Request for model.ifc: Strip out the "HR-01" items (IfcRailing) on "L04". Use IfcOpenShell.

First a look at what the model holds.

```python
import ifcopenshell
import ifcopenshell.util.element

model = ifcopenshell.open("model.ifc")
print(model.schema)
storey = next(s for s in model.by_type("IfcBuildingStorey") if s.Name == "L04")
railings = [e for e in ifcopenshell.util.element.get_decomposition(storey) if e.is_a("IfcRailing")]
seen = {}
for e in railings:
    element_type = ifcopenshell.util.element.get_type(e)
    name = element_type.Name if element_type not in (None, e) else None
    seen[name] = seen.get(name, 0) + 1
for name, count in sorted(seen.items(), key=str):
    print(count, "x", name)
```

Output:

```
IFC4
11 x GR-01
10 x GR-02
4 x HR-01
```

```python
import ifcopenshell
import ifcopenshell.api.root
import ifcopenshell.util.element

model = ifcopenshell.open("model.ifc")

storey = next(s for s in model.by_type("IfcBuildingStorey") if s.Name == "L04")
railings = [e for e in ifcopenshell.util.element.get_decomposition(storey) if e.is_a("IfcRailing")]
targets = [e for e in railings if (t := ifcopenshell.util.element.get_type(e)) not in (None, e) and t.Name == "HR-01"]

for e in targets:
    ifcopenshell.api.root.remove_product(model, product=e)
print(len(targets), "removed")

model.write("model_v2.ifc")
```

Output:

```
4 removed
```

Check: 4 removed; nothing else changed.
